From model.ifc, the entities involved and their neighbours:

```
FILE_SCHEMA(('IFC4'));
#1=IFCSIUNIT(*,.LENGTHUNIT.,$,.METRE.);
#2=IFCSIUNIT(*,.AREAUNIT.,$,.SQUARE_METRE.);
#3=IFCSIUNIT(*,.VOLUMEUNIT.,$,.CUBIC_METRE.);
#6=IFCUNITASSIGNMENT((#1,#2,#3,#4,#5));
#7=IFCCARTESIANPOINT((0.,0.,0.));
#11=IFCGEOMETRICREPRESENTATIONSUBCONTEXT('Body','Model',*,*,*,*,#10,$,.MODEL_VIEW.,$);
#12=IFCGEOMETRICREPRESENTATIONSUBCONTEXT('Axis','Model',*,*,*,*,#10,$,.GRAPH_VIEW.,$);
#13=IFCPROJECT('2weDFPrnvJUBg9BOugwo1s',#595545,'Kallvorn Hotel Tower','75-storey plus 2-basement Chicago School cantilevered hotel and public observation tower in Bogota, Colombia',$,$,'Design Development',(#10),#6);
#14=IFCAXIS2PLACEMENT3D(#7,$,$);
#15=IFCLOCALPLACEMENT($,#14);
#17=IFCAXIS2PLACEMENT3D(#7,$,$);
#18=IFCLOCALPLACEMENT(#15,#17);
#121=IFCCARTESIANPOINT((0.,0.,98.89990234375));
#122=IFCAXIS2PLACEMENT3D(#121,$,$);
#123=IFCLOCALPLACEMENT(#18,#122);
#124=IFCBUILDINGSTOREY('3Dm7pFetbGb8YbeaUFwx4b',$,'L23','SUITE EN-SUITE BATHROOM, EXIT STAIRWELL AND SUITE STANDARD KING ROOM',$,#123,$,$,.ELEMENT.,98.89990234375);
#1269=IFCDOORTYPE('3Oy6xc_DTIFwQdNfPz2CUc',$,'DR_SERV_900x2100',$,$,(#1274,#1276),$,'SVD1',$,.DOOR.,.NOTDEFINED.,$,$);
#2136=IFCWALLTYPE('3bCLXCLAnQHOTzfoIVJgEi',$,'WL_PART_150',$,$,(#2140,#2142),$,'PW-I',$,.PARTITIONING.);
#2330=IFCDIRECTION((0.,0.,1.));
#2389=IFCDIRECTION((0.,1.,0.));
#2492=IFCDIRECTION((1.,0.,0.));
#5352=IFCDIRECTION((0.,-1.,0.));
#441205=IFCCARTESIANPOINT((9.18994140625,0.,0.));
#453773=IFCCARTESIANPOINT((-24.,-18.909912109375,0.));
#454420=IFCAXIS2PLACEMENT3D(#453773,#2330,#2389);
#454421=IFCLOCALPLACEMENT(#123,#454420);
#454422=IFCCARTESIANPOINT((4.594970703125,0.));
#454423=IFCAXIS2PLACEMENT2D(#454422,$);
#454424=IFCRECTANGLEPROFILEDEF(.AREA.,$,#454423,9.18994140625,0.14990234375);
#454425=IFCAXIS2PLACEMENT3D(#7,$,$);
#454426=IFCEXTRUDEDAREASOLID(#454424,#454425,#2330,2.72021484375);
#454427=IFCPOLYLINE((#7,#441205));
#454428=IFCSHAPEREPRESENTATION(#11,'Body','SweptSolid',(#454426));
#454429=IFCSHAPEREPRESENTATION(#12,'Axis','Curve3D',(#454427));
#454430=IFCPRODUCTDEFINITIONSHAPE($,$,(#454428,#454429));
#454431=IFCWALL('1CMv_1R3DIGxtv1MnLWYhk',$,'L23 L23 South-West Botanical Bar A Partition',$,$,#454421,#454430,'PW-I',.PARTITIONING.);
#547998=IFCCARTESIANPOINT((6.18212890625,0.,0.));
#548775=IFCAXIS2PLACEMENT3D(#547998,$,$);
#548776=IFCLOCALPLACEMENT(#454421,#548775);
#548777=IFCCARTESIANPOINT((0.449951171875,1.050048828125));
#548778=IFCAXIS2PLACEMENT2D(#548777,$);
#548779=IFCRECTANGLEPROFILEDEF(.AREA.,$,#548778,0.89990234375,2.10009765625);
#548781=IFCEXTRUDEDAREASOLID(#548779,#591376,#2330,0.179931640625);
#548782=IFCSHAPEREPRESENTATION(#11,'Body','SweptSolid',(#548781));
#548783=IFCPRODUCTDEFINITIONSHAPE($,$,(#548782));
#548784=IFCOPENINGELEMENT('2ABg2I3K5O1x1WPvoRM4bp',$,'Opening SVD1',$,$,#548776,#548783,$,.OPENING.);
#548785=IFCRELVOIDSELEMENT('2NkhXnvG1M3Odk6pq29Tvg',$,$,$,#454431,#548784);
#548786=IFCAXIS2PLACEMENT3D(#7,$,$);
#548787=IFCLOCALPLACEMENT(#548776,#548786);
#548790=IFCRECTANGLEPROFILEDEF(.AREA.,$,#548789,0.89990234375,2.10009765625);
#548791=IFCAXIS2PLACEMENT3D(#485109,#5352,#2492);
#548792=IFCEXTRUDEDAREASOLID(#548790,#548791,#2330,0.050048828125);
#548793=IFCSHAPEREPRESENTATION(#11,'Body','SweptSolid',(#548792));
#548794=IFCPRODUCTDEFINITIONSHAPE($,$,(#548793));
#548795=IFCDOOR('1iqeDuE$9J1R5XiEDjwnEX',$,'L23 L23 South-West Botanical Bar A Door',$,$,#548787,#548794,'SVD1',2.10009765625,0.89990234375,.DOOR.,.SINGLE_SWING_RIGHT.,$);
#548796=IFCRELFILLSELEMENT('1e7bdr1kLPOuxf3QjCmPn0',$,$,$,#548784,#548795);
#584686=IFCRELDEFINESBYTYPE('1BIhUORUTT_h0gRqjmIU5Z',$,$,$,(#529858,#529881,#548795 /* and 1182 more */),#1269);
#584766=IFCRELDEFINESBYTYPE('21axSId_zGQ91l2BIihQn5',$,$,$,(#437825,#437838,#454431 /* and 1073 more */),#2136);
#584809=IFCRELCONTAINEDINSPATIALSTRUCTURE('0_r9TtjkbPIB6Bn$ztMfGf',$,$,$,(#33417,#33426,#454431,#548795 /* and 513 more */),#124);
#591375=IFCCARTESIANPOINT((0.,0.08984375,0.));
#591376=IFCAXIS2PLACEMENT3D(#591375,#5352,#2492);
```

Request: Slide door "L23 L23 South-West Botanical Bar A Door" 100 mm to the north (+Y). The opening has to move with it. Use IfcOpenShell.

```python
import ifcopenshell
import ifcopenshell.api.geometry
import ifcopenshell.util.placement
import ifcopenshell.util.unit

model = ifcopenshell.open("model.ifc")
unit_scale = ifcopenshell.util.unit.calculate_unit_scale(model)

door = model.by_guid("1iqeDuE$9J1R5XiEDjwnEX")
opening = door.FillsVoids[0].RelatingOpeningElement
wall = opening.VoidsElements[0].RelatingBuildingElement

wall_matrix = ifcopenshell.util.placement.get_local_placement(wall.ObjectPlacement)
shift = wall_matrix[:3, 0] * 0.1 / unit_scale
before = ifcopenshell.util.placement.get_local_placement(door.ObjectPlacement)[:3, 3].copy()

# The door is placed relative to its opening, so it follows when the opening moves.
matrix = ifcopenshell.util.placement.get_local_placement(opening.ObjectPlacement)
matrix[:3, 3] += shift
ifcopenshell.api.geometry.edit_object_placement(
    model, product=opening, matrix=matrix, is_si=False, should_transform_children=True
)

after = ifcopenshell.util.placement.get_local_placement(door.ObjectPlacement)[:3, 3]
print("door moved by", (after - before).round(3) + 0.0)

model.write("model_v2.ifc")
```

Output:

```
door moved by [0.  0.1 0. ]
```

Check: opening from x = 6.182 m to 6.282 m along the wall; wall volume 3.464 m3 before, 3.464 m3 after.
